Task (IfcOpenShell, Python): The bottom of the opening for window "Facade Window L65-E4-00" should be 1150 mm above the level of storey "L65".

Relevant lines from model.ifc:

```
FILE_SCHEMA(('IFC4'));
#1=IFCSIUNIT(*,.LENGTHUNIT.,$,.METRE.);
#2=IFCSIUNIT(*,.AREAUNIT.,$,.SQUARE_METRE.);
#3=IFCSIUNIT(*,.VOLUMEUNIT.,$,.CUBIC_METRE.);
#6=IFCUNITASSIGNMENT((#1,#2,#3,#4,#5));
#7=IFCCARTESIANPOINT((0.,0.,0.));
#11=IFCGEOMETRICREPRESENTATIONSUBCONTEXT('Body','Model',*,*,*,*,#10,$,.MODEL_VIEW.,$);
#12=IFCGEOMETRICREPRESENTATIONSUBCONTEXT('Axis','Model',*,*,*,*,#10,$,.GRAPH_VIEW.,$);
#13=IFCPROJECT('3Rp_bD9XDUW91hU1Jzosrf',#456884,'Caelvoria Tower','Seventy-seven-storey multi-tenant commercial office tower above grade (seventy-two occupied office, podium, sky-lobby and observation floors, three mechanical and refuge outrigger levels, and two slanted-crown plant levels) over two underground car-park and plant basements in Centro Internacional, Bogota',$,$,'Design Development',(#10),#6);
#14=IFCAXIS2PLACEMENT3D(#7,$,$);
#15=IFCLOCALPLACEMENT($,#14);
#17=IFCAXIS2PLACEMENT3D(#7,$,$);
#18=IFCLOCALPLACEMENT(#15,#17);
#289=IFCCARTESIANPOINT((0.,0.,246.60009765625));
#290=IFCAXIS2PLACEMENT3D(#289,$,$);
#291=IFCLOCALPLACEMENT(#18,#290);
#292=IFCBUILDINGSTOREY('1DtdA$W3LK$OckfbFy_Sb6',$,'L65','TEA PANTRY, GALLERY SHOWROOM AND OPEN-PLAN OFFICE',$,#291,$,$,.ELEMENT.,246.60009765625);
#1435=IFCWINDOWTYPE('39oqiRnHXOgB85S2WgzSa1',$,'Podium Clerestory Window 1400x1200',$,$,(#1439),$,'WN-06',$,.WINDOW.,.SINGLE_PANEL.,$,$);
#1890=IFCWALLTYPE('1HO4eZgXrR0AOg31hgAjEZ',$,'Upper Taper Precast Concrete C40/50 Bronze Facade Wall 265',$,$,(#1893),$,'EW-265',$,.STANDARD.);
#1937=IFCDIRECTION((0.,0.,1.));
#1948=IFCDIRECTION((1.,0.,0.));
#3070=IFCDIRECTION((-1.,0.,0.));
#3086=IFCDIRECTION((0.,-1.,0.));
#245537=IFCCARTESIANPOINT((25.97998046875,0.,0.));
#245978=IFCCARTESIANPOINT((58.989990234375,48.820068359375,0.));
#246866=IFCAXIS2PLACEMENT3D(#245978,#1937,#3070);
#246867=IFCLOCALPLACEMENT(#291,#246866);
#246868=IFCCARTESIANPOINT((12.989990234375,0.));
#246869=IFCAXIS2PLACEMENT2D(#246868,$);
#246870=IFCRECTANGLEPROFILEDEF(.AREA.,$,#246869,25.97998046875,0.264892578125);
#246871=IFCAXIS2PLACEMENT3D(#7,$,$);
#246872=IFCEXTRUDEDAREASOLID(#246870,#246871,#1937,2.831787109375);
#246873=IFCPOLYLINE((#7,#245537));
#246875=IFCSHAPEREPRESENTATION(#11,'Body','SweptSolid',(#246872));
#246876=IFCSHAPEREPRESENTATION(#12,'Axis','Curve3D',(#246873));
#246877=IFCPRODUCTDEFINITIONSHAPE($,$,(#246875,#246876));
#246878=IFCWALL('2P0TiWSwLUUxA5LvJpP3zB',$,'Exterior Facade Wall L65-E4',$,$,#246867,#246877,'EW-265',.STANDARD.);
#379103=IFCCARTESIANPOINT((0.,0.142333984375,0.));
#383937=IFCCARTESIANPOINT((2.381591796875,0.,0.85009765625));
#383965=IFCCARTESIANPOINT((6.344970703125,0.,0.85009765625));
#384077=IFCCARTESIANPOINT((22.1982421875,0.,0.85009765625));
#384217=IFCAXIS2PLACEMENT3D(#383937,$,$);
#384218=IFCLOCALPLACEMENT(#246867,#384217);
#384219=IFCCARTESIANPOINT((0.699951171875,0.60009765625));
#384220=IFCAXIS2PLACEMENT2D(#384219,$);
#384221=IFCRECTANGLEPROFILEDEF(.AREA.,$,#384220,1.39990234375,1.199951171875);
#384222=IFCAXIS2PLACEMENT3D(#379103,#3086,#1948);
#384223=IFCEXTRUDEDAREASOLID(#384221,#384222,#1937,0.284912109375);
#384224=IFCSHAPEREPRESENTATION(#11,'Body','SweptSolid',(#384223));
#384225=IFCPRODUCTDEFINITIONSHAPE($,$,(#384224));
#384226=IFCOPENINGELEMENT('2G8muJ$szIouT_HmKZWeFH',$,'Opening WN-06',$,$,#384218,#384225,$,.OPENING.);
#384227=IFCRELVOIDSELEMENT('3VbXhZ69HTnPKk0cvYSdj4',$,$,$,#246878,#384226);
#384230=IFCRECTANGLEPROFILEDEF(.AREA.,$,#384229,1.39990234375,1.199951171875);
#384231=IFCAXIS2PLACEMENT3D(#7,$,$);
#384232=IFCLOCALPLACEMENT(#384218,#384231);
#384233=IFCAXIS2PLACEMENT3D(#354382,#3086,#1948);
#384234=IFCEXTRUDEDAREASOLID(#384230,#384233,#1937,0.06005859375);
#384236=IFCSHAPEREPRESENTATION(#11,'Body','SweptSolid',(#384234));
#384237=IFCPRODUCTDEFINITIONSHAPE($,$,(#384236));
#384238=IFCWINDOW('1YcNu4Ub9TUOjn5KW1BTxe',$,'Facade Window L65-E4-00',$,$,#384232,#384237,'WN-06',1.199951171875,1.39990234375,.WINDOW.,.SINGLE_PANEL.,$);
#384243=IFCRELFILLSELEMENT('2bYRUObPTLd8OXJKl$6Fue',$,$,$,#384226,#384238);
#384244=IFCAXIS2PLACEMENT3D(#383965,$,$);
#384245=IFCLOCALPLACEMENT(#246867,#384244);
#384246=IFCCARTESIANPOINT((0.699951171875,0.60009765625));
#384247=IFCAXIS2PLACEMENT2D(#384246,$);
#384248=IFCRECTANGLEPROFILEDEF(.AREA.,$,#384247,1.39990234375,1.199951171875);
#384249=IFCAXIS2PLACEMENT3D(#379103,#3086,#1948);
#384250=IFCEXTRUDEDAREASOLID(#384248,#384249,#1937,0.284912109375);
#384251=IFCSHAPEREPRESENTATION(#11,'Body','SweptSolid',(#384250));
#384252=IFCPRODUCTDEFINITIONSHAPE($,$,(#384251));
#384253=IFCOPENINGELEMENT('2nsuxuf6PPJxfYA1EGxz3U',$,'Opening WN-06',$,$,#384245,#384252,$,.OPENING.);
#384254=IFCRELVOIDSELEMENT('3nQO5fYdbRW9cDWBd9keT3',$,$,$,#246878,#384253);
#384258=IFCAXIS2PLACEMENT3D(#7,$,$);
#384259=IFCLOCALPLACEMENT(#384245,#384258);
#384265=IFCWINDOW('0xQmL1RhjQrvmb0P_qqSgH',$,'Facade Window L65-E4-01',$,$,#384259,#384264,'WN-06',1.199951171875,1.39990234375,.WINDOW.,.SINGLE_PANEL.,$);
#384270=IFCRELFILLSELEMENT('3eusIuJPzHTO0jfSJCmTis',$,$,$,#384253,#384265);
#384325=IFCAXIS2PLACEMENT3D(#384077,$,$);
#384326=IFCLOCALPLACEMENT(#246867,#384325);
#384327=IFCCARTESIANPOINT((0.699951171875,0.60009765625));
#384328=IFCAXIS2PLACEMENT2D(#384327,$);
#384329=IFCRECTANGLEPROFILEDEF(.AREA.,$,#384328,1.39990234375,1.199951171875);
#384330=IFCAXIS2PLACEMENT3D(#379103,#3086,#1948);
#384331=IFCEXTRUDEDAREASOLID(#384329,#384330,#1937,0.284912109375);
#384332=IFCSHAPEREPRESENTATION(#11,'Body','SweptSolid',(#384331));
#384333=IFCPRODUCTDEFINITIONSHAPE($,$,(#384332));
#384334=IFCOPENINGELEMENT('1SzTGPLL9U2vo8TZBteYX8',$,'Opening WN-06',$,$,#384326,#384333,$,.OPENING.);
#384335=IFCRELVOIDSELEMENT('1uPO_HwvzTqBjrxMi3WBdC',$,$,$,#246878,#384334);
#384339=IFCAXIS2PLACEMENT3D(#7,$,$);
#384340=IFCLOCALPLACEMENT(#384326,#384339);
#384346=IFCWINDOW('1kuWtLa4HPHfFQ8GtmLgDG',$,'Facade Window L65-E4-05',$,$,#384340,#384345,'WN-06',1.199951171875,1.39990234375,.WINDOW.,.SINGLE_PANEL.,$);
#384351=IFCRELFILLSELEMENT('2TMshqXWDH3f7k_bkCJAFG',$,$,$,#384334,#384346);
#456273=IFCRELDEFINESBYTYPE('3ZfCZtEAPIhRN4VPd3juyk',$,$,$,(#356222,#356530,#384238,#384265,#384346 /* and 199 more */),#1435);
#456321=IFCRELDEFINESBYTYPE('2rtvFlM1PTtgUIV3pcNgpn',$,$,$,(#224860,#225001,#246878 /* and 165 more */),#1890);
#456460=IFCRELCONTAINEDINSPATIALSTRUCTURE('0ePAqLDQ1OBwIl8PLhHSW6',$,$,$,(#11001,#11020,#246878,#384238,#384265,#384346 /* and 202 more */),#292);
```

```python
import numpy as np
import ifcopenshell
import ifcopenshell.api.geometry
import ifcopenshell.geom
import ifcopenshell.util.element
import ifcopenshell.util.placement
import ifcopenshell.util.shape
import ifcopenshell.util.unit

model = ifcopenshell.open("model.ifc")
unit_scale = ifcopenshell.util.unit.calculate_unit_scale(model)

window = model.by_guid("1YcNu4Ub9TUOjn5KW1BTxe")
opening = window.FillsVoids[0].RelatingOpeningElement
storey = ifcopenshell.util.element.get_container(window, ifc_class="IfcBuildingStorey")
level = ifcopenshell.util.placement.get_local_placement(storey.ObjectPlacement)[2, 3]

# The opening's origin need not be at the sill, so measure its lowest point.
shape = ifcopenshell.geom.create_shape(ifcopenshell.geom.settings(), opening)
bottom = ifcopenshell.util.shape.get_shape_bottom_elevation(shape, shape.geometry) / unit_scale
dz = level + 1.15 - bottom

shift = np.array([0.0, 0.0, dz])
# The window is placed relative to its opening, so it follows when the opening moves.
matrix = ifcopenshell.util.placement.get_local_placement(opening.ObjectPlacement)
matrix[:3, 3] += shift
ifcopenshell.api.geometry.edit_object_placement(
    model, product=opening, matrix=matrix, is_si=False, should_transform_children=True
)

print(f"moved by {dz * unit_scale:+.3f} m")

model.write("model-out.ifc")
```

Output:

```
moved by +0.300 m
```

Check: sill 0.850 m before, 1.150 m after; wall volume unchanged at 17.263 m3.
